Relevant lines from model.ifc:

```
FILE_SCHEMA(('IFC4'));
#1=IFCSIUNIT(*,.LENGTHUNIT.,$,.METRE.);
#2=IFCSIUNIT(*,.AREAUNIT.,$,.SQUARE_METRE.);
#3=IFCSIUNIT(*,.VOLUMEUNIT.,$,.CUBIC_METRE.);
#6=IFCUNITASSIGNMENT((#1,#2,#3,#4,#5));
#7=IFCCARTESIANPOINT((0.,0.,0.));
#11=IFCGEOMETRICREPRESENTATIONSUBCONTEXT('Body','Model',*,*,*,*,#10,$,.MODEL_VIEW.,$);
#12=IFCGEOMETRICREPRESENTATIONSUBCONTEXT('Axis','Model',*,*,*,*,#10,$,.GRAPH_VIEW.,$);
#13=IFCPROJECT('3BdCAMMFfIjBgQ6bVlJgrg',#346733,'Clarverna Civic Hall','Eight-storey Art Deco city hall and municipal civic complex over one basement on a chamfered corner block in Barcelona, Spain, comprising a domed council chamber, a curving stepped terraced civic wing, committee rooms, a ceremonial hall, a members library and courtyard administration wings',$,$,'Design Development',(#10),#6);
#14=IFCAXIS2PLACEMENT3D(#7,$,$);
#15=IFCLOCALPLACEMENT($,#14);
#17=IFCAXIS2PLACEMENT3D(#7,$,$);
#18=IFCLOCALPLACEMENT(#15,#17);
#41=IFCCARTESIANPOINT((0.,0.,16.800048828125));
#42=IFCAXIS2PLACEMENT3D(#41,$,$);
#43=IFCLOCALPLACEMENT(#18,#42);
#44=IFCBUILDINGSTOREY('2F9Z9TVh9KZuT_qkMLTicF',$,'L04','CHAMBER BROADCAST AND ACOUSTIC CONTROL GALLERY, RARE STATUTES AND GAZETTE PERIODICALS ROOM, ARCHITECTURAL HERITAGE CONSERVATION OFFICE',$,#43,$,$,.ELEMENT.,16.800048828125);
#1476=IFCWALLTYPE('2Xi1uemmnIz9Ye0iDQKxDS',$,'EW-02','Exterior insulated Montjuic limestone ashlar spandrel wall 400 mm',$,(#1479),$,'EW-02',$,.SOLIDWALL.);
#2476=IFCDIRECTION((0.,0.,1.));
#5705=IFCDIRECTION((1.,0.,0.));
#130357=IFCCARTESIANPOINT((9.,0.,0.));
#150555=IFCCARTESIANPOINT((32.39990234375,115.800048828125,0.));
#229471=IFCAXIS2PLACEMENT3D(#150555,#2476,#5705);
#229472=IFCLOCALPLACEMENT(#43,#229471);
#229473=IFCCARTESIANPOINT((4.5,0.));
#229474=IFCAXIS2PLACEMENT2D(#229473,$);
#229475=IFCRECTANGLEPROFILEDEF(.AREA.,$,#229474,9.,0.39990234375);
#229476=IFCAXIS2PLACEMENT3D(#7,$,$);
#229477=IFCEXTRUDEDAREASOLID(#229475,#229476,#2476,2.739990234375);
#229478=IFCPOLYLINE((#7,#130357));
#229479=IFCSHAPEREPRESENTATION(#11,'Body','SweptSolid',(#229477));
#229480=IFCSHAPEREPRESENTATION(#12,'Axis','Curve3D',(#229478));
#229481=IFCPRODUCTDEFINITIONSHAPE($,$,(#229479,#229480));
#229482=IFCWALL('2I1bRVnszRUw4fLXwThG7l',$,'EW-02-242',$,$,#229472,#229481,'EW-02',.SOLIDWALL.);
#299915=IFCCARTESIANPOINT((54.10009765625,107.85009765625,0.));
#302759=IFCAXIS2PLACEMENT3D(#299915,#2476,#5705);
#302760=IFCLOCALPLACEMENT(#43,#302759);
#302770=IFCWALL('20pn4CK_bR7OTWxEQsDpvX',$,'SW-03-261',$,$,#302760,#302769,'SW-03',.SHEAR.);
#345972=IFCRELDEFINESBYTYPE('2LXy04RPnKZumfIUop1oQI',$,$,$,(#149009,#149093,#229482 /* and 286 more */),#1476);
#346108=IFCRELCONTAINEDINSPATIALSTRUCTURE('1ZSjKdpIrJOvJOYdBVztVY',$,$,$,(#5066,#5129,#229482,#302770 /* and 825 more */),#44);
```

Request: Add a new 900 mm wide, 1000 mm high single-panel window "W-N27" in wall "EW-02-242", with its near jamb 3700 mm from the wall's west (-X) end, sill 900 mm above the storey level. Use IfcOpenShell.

```python
import numpy as np
import ifcopenshell
import ifcopenshell.api.feature
import ifcopenshell.api.geometry
import ifcopenshell.api.root
import ifcopenshell.api.spatial
import ifcopenshell.geom
import ifcopenshell.util.element
import ifcopenshell.util.placement
import ifcopenshell.util.representation
import ifcopenshell.util.shape
import ifcopenshell.util.unit

model = ifcopenshell.open("model.ifc")
unit_scale = ifcopenshell.util.unit.calculate_unit_scale(model)
settings = ifcopenshell.geom.settings()


def volume(element):
    """Net volume in cubic metres, openings subtracted."""
    shape = ifcopenshell.geom.create_shape(settings, element)
    return ifcopenshell.util.shape.get_volume(shape.geometry)


wall = model.by_guid("2I1bRVnszRUw4fLXwThG7l")
storey = ifcopenshell.util.element.get_container(wall, ifc_class="IfcBuildingStorey")
context = ifcopenshell.util.representation.get_context(model, "Model", "Body", "MODEL_VIEW")
before = volume(wall)

width, height, from_end, sill = 0.9, 1, 3.7, 0.9  # metres

# The wall runs along its own X axis, and the end named is its -X end.
wall_shape = ifcopenshell.geom.create_shape(settings, wall)
x, y, z = ifcopenshell.util.shape.get_vertices(wall_shape.geometry).T
start = x.min() + from_end
face, thickness = float(y.min()), float(y.max() - y.min())
wall_matrix = ifcopenshell.util.placement.get_local_placement(wall.ObjectPlacement)
level = ifcopenshell.util.placement.get_local_placement(storey.ObjectPlacement)[2, 3]


def in_wall(x, y):
    """Placement at x, y metres in the wall's axes, at sill height."""
    matrix = wall_matrix.copy()
    matrix[:, 3] = wall_matrix @ np.array([x / unit_scale, y / unit_scale, 0.0, 1.0])
    matrix[2, 3] = level + sill / unit_scale
    return matrix


# Opening: a box that overshoots both wall faces by 50 mm.
opening = ifcopenshell.api.root.create_entity(model, ifc_class="IfcOpeningElement", predefined_type="OPENING")
box = ifcopenshell.api.geometry.add_wall_representation(
    model, context=context, length=width, height=height, thickness=thickness + 0.1
)
ifcopenshell.api.geometry.assign_representation(model, product=opening, representation=box)
ifcopenshell.api.geometry.edit_object_placement(model, product=opening, matrix=in_wall(start, face - 0.05), is_si=False)
ifcopenshell.api.feature.add_feature(model, feature=opening, element=wall)

window = ifcopenshell.api.root.create_entity(model, ifc_class="IfcWindow", name="W-N27", predefined_type="WINDOW")
window.OverallWidth, window.OverallHeight = width / unit_scale, height / unit_scale
window.PartitioningType = "SINGLE_PANEL"
body = ifcopenshell.api.geometry.add_window_representation(
    model,
    context=context,
    overall_width=window.OverallWidth,
    overall_height=window.OverallHeight,
    partition_type="SINGLE_PANEL",
)
ifcopenshell.api.geometry.assign_representation(model, product=window, representation=body)
ifcopenshell.api.spatial.assign_container(model, products=[window], relating_structure=storey)
ifcopenshell.api.feature.add_filling(model, opening=opening, element=window)

# Centre the window in the wall's thickness.
ifcopenshell.api.geometry.edit_object_placement(model, product=window, matrix=in_wall(start, face), is_si=False)
window_shape = ifcopenshell.geom.create_shape(settings, window)
depth = ifcopenshell.util.shape.get_vertices(window_shape.geometry)[:, 1]
offset = face + thickness / 2 - (depth.min() + depth.max()) / 2
ifcopenshell.api.geometry.edit_object_placement(model, product=window, matrix=in_wall(start, offset), is_si=False)

after = volume(wall)

print(f"wall volume {before:.3f} -> {after:.3f} m3")

model.write("model_edited.ifc")
```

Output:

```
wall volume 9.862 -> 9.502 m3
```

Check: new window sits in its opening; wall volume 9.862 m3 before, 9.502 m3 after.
